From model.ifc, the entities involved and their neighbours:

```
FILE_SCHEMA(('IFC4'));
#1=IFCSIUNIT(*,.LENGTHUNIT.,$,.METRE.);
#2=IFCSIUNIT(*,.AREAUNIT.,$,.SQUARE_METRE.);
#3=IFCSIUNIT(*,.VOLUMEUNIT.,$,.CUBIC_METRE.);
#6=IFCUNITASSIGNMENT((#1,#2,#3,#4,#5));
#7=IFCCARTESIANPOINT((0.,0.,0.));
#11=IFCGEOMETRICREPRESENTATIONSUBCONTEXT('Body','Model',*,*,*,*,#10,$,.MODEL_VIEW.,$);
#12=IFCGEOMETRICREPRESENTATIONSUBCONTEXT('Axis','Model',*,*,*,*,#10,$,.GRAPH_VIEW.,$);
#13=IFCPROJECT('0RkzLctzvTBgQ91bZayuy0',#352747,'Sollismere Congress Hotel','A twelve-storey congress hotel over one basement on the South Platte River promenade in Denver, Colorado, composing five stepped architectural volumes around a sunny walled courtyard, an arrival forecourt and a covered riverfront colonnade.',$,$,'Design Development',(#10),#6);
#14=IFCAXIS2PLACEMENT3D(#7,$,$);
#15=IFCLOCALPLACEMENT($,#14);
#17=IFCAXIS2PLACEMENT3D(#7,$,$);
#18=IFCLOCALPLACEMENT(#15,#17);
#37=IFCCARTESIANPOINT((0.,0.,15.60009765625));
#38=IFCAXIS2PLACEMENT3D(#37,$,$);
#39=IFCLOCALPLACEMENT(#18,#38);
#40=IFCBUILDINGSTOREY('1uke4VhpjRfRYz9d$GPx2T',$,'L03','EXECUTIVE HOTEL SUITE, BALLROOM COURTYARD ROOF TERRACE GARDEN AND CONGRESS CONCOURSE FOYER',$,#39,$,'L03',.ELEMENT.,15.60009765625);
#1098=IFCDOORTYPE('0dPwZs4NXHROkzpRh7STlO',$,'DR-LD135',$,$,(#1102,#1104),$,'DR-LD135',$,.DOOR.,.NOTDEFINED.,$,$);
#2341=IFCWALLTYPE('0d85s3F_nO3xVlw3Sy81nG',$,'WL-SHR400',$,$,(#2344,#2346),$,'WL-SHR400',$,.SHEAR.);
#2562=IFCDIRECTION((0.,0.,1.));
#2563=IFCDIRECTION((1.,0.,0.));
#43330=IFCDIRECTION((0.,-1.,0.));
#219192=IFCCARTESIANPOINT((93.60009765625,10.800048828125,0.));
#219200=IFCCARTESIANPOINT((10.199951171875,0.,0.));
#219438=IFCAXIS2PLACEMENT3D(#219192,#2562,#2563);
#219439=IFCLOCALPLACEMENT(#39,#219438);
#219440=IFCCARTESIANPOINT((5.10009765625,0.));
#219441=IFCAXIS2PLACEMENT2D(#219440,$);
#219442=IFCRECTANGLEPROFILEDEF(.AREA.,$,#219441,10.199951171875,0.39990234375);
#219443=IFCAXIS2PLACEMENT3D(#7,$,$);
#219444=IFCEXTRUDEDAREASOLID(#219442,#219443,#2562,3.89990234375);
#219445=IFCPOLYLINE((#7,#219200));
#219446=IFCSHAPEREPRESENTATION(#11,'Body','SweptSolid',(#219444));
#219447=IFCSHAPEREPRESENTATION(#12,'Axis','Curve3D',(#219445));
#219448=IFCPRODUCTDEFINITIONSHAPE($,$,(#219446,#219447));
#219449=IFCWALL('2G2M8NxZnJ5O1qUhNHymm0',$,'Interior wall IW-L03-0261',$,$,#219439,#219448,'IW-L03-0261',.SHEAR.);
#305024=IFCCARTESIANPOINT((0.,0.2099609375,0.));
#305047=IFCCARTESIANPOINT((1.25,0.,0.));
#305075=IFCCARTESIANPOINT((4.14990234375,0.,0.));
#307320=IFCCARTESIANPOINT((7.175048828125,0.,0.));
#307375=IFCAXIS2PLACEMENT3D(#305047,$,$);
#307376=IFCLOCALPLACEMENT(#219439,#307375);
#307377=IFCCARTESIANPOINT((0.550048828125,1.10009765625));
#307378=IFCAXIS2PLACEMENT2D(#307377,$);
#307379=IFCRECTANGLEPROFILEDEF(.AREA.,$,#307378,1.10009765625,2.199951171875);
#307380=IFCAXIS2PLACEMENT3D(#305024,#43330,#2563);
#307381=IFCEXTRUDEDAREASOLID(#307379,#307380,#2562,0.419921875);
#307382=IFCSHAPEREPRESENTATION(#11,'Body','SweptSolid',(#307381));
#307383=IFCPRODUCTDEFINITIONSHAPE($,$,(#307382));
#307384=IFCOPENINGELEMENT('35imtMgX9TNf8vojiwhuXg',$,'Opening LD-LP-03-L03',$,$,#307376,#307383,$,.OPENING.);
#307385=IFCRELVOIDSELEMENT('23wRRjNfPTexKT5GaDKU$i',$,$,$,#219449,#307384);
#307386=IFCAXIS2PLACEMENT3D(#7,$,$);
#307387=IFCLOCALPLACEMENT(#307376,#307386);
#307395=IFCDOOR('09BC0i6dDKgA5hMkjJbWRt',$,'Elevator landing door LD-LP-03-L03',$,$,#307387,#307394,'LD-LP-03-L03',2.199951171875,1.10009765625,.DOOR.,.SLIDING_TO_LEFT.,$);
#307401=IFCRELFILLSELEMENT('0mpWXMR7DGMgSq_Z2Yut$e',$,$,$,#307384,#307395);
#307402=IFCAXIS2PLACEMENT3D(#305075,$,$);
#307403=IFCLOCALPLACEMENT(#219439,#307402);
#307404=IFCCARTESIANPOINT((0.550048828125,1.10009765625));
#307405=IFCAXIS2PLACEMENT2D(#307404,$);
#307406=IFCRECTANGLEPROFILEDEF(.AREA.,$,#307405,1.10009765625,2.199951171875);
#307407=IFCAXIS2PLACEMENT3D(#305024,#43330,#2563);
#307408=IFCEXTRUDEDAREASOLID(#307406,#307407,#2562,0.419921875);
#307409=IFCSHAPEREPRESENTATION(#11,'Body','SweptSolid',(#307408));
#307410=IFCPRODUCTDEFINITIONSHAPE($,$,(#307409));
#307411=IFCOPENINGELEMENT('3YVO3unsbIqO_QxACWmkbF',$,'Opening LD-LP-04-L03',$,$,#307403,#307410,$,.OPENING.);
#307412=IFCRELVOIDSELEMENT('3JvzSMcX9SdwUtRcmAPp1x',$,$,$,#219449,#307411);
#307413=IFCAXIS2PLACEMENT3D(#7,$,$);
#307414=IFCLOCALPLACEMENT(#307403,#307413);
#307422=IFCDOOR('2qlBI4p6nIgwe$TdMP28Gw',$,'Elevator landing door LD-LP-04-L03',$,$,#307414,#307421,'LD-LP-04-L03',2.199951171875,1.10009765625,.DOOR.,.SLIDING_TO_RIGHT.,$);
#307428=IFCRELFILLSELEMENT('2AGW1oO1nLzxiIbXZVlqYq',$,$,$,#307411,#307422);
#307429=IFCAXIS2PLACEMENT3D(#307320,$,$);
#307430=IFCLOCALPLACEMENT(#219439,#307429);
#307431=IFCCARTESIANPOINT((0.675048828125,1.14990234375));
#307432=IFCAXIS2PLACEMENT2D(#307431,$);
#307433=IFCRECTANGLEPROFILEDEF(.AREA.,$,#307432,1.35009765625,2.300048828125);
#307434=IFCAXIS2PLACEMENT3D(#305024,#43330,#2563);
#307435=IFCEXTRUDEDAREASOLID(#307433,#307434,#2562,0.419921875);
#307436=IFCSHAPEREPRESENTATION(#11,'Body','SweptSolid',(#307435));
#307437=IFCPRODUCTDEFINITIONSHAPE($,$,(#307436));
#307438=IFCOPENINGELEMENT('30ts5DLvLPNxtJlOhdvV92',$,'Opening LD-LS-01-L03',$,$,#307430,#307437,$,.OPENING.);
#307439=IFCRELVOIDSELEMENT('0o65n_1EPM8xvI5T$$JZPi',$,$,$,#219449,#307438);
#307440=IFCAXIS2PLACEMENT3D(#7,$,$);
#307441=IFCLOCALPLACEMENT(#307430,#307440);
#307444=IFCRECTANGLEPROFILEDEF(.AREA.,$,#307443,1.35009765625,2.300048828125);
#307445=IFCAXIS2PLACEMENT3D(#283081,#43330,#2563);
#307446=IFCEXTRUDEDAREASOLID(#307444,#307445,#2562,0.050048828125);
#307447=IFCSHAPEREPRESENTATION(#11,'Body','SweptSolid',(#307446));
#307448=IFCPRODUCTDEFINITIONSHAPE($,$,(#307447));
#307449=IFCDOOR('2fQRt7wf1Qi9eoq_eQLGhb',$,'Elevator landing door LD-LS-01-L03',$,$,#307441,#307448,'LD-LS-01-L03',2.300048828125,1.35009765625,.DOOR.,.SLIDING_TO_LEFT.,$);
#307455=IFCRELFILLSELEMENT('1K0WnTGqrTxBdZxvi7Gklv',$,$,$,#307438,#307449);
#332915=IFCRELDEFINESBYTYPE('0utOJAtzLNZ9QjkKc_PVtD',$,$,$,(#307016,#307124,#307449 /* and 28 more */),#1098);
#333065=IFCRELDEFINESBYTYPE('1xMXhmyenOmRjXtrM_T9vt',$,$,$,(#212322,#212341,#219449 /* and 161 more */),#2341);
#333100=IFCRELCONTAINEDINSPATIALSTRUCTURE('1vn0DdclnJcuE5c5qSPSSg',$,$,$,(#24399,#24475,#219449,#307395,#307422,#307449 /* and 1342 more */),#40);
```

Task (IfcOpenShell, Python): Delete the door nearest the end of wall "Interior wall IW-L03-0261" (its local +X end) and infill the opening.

```python
import ifcopenshell
import ifcopenshell.api.feature
import ifcopenshell.api.root
import ifcopenshell.geom
import ifcopenshell.util.shape

model = ifcopenshell.open("model.ifc")
settings = ifcopenshell.geom.settings()


def volume(element):
    """Net volume in cubic metres, openings subtracted."""
    shape = ifcopenshell.geom.create_shape(settings, element)
    return ifcopenshell.util.shape.get_volume(shape.geometry)


door = model.by_guid("2fQRt7wf1Qi9eoq_eQLGhb")
opening = door.FillsVoids[0].RelatingOpeningElement
wall = opening.VoidsElements[0].RelatingBuildingElement
before = volume(wall)

ifcopenshell.api.root.remove_product(model, product=door)
ifcopenshell.api.feature.remove_feature(model, feature=opening)

after = volume(wall)

print(f"wall volume {before:.3f} -> {after:.3f} m3")

model.write("model_v2.ifc")
```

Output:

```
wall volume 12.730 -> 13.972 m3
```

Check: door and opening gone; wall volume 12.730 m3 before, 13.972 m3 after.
